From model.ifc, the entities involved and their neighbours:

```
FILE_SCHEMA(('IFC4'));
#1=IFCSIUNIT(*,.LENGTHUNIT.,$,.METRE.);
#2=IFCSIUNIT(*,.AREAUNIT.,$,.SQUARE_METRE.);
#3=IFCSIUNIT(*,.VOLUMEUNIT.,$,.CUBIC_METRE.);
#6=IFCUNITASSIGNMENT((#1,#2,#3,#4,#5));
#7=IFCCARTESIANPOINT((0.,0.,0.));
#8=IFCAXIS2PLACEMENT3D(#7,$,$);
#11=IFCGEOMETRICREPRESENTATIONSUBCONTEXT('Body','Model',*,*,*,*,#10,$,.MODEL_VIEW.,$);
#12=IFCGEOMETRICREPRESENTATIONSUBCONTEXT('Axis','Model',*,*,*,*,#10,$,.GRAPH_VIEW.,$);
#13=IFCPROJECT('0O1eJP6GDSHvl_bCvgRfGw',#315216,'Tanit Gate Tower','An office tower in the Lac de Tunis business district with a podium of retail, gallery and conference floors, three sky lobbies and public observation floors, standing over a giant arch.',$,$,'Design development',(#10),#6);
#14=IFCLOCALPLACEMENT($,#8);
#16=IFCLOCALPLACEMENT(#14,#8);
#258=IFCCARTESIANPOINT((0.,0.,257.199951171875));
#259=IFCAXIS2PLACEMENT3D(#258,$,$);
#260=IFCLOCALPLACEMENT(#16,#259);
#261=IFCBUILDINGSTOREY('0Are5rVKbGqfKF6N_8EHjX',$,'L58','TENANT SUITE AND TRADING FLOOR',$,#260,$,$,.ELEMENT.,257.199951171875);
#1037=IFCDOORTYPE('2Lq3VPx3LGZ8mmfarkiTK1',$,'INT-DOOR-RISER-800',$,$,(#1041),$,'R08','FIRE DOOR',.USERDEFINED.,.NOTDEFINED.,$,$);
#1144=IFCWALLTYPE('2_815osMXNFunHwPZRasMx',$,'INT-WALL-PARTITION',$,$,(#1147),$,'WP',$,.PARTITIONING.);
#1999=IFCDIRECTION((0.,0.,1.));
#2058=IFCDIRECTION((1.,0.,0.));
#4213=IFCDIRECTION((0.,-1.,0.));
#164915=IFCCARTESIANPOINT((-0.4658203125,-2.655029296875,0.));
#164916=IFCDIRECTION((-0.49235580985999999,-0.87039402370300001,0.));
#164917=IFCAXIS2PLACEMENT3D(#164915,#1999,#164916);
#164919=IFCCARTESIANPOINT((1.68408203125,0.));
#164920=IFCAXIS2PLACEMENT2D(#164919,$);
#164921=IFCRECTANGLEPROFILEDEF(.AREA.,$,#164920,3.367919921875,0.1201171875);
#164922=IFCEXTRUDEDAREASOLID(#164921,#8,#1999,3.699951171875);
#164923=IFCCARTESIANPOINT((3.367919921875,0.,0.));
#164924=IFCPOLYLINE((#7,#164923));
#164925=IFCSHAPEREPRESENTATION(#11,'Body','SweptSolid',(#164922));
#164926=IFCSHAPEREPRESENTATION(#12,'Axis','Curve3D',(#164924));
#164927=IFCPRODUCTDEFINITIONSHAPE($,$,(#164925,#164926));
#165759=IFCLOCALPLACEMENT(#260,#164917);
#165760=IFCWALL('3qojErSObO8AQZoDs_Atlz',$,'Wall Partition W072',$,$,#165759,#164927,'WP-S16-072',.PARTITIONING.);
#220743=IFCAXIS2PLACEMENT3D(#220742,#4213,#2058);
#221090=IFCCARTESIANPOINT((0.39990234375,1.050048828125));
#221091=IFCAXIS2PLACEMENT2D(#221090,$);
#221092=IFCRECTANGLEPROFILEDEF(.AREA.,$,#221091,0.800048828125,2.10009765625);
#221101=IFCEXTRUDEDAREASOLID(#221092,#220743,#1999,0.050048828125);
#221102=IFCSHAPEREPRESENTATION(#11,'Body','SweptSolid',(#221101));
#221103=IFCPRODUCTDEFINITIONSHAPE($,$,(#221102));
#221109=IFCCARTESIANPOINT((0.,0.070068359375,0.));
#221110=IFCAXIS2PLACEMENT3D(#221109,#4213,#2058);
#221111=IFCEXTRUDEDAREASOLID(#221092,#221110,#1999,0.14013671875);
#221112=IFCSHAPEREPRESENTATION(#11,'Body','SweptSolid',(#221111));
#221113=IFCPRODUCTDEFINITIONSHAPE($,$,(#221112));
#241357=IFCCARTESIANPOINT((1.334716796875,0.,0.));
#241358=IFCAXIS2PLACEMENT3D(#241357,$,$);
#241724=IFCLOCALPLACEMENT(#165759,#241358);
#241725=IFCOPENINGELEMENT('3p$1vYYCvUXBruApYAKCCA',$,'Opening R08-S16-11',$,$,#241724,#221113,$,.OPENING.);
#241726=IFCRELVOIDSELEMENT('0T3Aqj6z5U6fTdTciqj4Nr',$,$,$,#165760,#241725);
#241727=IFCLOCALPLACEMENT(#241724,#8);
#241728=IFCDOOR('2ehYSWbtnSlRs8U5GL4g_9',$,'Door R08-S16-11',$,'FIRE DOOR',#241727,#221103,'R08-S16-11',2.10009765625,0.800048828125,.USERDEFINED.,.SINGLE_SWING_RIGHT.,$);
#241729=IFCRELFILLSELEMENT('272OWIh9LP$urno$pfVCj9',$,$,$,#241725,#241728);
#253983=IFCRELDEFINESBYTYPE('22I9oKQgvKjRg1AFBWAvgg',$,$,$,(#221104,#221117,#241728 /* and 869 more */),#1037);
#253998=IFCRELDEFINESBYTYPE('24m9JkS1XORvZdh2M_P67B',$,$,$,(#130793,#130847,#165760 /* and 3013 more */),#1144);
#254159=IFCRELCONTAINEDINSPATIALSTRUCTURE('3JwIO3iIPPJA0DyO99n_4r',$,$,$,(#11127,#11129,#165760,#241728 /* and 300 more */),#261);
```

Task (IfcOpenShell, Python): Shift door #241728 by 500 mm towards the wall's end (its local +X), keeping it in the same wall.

```python
import ifcopenshell
import ifcopenshell.api.geometry
import ifcopenshell.util.placement
import ifcopenshell.util.unit

model = ifcopenshell.open("model.ifc")
unit_scale = ifcopenshell.util.unit.calculate_unit_scale(model)

door = model.by_guid("2ehYSWbtnSlRs8U5GL4g_9")
opening = door.FillsVoids[0].RelatingOpeningElement
wall = opening.VoidsElements[0].RelatingBuildingElement

wall_matrix = ifcopenshell.util.placement.get_local_placement(wall.ObjectPlacement)
shift = wall_matrix[:3, 0] * 0.5 / unit_scale
before = ifcopenshell.util.placement.get_local_placement(door.ObjectPlacement)[:3, 3].copy()

# The door is placed relative to its opening, so it follows when the opening moves.
matrix = ifcopenshell.util.placement.get_local_placement(opening.ObjectPlacement)
matrix[:3, 3] += shift
ifcopenshell.api.geometry.edit_object_placement(
    model, product=opening, matrix=matrix, is_si=False, should_transform_children=True
)

after = ifcopenshell.util.placement.get_local_placement(door.ObjectPlacement)[:3, 3]
print("door moved by", (after - before).round(3) + 0.0)

model.write("model-out.ifc")
```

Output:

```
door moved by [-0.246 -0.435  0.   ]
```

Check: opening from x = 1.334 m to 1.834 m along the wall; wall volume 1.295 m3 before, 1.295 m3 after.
